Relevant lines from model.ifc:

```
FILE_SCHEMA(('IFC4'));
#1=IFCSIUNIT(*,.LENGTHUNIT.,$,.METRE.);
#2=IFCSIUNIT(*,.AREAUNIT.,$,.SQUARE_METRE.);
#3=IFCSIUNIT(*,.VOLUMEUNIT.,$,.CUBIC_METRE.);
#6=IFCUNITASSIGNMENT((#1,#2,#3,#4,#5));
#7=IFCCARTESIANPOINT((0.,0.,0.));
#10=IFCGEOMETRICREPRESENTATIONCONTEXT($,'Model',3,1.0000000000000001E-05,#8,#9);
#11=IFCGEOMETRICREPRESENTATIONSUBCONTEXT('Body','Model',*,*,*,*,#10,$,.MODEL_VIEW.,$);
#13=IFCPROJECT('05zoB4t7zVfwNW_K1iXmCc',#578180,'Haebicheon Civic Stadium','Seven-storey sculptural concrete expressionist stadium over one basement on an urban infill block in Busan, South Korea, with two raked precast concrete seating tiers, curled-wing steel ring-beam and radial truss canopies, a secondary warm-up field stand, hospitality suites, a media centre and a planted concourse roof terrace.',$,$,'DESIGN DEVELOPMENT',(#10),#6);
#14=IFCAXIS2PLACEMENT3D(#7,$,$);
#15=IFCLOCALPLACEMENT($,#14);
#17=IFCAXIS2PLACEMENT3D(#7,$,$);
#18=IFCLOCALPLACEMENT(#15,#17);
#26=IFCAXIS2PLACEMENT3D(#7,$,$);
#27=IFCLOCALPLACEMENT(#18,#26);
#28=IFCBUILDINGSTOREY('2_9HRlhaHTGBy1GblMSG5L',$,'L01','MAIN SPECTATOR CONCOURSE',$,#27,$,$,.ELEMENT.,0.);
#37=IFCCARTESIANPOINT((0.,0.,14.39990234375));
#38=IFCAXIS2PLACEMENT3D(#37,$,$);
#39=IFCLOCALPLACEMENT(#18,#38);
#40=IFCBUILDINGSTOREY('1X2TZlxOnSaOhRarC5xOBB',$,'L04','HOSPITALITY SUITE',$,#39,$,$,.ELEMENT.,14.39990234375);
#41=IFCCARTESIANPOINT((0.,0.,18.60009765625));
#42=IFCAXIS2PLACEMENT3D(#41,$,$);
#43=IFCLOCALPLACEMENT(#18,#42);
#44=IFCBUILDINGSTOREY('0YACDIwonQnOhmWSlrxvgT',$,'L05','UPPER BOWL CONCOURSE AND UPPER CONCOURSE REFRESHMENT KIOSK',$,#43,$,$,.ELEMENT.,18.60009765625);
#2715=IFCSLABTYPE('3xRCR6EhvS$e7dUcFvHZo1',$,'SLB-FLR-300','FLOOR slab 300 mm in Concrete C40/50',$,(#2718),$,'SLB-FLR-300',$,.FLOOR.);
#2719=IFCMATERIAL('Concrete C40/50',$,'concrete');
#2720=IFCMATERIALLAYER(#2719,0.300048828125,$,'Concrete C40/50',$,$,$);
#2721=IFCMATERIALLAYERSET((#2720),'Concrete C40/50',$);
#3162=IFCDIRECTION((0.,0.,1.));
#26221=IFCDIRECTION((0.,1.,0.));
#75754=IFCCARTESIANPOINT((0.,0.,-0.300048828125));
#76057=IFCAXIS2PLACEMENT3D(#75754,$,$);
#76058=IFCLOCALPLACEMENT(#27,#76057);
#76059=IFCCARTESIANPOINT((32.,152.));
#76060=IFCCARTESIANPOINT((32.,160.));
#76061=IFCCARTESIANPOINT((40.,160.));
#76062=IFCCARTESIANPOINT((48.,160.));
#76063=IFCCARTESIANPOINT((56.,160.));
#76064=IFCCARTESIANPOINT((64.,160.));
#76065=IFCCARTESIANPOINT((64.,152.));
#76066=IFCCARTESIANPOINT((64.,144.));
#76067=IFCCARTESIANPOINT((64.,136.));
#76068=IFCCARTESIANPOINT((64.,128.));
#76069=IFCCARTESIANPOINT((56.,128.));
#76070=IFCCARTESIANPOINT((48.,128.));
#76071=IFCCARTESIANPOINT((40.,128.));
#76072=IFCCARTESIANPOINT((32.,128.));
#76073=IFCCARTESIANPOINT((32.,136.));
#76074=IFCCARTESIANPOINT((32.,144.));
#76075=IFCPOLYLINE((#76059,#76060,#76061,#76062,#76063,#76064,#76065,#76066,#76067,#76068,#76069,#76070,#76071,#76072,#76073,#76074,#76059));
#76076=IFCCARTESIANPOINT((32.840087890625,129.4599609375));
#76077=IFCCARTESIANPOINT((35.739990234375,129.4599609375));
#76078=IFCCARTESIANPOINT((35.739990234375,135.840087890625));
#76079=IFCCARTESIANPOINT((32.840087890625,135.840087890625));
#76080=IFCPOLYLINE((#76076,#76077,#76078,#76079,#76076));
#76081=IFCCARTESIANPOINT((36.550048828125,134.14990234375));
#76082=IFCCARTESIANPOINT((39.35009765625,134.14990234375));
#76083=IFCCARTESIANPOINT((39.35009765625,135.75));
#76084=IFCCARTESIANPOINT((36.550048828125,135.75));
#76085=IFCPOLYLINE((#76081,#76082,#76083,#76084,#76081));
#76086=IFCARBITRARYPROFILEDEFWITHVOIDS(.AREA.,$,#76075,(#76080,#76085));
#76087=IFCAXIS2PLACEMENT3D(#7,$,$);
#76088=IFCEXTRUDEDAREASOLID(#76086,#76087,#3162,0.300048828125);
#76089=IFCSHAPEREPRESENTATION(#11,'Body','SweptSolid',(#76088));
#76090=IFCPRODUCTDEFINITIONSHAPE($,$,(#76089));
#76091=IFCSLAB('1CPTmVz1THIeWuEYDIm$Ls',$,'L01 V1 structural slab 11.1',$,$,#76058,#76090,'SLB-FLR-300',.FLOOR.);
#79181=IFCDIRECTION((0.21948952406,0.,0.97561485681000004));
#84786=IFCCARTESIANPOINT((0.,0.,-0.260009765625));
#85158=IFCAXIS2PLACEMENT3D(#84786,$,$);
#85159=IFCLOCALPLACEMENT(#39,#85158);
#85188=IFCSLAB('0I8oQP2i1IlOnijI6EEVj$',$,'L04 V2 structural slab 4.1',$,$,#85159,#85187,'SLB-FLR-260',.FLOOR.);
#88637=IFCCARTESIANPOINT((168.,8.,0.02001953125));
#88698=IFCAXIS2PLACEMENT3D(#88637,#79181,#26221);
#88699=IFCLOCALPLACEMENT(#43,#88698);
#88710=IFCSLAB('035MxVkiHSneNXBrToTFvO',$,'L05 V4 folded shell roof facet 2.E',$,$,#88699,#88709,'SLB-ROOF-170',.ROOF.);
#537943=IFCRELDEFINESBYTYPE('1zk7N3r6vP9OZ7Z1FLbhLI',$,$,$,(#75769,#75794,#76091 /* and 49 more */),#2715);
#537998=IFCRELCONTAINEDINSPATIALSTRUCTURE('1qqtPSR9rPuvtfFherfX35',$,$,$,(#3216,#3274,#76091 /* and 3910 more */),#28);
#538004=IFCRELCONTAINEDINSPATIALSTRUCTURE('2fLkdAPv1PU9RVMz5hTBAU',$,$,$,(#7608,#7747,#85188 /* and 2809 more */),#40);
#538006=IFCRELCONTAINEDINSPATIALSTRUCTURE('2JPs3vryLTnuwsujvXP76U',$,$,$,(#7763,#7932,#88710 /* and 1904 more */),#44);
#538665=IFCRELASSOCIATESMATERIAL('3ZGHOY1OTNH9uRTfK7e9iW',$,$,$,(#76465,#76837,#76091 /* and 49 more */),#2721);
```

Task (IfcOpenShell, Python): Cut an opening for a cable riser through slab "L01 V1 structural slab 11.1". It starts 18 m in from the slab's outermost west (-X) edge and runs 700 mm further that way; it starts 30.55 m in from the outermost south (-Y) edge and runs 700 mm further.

```python
import numpy as np
import ifcopenshell
import ifcopenshell.api.feature
import ifcopenshell.api.geometry
import ifcopenshell.api.root
import ifcopenshell.geom
import ifcopenshell.util.placement
import ifcopenshell.util.representation
import ifcopenshell.util.shape
import ifcopenshell.util.unit

model = ifcopenshell.open("model.ifc")
unit_scale = ifcopenshell.util.unit.calculate_unit_scale(model)
settings = ifcopenshell.geom.settings()


def volume(element):
    """Net volume in cubic metres, openings subtracted."""
    shape = ifcopenshell.geom.create_shape(settings, element)
    return ifcopenshell.util.shape.get_volume(shape.geometry)


slab = model.by_guid("1CPTmVz1THIeWuEYDIm$Ls")
before = volume(slab)

# Extent in the slab's own axes, in metres. The edges named are its -X and -Y sides.
slab_shape = ifcopenshell.geom.create_shape(settings, slab)
vertices = ifcopenshell.util.shape.get_vertices(slab_shape.geometry)
x_min, y_min, bottom = vertices.min(axis=0)
top = vertices[:, 2].max()

opening = ifcopenshell.api.root.create_entity(model, ifc_class="IfcOpeningElement", name="Cable riser opening", predefined_type="OPENING")
context = ifcopenshell.util.representation.get_context(model, "Model", "Body", "MODEL_VIEW")
width, depth = 0.7, 0.7
outline = [(0.0, 0.0), (width, 0.0), (width, depth), (0.0, depth), (0.0, 0.0)]
# Overshoot both faces by 50 mm so the cut is clean.
shape = ifcopenshell.api.geometry.add_slab_representation(
    model, context=context, depth=top - bottom + 0.1, polyline=outline
)
ifcopenshell.api.geometry.assign_representation(model, product=opening, representation=shape)

matrix = ifcopenshell.util.placement.get_local_placement(slab.ObjectPlacement)
matrix[:, 3] = matrix @ np.append(np.array([x_min + 18, y_min + 30.55, bottom - 0.05]) / unit_scale, 1.0)
ifcopenshell.api.geometry.edit_object_placement(model, product=opening, matrix=matrix, is_si=False)
ifcopenshell.api.feature.add_feature(model, feature=opening, element=slab)

after = volume(slab)

print(f"slab volume {before:.3f} -> {after:.3f} m3")

model.write("model_edited.ifc")
```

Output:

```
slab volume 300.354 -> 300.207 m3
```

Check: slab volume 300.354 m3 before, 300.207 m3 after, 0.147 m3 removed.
